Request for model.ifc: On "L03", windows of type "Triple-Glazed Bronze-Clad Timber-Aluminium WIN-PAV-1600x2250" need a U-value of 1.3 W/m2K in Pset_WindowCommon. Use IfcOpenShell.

First a look at what the model holds.

```python
import ifcopenshell
import ifcopenshell.util.element

model = ifcopenshell.open("model.ifc")
print(model.schema)
storey = next(s for s in model.by_type("IfcBuildingStorey") if s.Name == "L03")
windows = [e for e in ifcopenshell.util.element.get_decomposition(storey) if e.is_a("IfcWindow")]
seen = {}
for e in windows:
    element_type = ifcopenshell.util.element.get_type(e)
    key = (element_type.Name if element_type != e and element_type else None, ifcopenshell.util.element.get_pset(e, "Pset_WindowCommon", "ThermalTransmittance"))
    seen[key] = seen.get(key, 0) + 1
for (name, value), count in sorted(seen.items(), key=str):
    print(count, "x", name, "|", value)
```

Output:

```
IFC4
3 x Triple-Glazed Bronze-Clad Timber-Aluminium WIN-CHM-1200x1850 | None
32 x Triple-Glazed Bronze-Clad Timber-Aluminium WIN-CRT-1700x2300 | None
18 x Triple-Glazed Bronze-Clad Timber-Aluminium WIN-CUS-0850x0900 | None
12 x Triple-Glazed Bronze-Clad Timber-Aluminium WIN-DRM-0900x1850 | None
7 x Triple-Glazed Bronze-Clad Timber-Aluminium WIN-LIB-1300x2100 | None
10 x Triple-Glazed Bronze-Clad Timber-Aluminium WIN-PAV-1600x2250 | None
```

```python
import ifcopenshell
import ifcopenshell.api.pset
import ifcopenshell.util.element

model = ifcopenshell.open("model.ifc")

storey = next(s for s in model.by_type("IfcBuildingStorey") if s.Name == "L03")
windows = [e for e in ifcopenshell.util.element.get_decomposition(storey) if e.is_a("IfcWindow")]

count = 0
for e in windows:
    element_type = ifcopenshell.util.element.get_type(e)
    if element_type in (None, e) or element_type.Name != "Triple-Glazed Bronze-Clad Timber-Aluminium WIN-PAV-1600x2250":
        continue
    # add_pset returns the element's existing set when there is one.
    pset = ifcopenshell.api.pset.add_pset(model, product=e, name="Pset_WindowCommon")
    ifcopenshell.api.pset.edit_pset(model, pset=pset, properties={"ThermalTransmittance": 1.3})
    count += 1

print(count, "windows updated")

model.write("model_v2.ifc")
```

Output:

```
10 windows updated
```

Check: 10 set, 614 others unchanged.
